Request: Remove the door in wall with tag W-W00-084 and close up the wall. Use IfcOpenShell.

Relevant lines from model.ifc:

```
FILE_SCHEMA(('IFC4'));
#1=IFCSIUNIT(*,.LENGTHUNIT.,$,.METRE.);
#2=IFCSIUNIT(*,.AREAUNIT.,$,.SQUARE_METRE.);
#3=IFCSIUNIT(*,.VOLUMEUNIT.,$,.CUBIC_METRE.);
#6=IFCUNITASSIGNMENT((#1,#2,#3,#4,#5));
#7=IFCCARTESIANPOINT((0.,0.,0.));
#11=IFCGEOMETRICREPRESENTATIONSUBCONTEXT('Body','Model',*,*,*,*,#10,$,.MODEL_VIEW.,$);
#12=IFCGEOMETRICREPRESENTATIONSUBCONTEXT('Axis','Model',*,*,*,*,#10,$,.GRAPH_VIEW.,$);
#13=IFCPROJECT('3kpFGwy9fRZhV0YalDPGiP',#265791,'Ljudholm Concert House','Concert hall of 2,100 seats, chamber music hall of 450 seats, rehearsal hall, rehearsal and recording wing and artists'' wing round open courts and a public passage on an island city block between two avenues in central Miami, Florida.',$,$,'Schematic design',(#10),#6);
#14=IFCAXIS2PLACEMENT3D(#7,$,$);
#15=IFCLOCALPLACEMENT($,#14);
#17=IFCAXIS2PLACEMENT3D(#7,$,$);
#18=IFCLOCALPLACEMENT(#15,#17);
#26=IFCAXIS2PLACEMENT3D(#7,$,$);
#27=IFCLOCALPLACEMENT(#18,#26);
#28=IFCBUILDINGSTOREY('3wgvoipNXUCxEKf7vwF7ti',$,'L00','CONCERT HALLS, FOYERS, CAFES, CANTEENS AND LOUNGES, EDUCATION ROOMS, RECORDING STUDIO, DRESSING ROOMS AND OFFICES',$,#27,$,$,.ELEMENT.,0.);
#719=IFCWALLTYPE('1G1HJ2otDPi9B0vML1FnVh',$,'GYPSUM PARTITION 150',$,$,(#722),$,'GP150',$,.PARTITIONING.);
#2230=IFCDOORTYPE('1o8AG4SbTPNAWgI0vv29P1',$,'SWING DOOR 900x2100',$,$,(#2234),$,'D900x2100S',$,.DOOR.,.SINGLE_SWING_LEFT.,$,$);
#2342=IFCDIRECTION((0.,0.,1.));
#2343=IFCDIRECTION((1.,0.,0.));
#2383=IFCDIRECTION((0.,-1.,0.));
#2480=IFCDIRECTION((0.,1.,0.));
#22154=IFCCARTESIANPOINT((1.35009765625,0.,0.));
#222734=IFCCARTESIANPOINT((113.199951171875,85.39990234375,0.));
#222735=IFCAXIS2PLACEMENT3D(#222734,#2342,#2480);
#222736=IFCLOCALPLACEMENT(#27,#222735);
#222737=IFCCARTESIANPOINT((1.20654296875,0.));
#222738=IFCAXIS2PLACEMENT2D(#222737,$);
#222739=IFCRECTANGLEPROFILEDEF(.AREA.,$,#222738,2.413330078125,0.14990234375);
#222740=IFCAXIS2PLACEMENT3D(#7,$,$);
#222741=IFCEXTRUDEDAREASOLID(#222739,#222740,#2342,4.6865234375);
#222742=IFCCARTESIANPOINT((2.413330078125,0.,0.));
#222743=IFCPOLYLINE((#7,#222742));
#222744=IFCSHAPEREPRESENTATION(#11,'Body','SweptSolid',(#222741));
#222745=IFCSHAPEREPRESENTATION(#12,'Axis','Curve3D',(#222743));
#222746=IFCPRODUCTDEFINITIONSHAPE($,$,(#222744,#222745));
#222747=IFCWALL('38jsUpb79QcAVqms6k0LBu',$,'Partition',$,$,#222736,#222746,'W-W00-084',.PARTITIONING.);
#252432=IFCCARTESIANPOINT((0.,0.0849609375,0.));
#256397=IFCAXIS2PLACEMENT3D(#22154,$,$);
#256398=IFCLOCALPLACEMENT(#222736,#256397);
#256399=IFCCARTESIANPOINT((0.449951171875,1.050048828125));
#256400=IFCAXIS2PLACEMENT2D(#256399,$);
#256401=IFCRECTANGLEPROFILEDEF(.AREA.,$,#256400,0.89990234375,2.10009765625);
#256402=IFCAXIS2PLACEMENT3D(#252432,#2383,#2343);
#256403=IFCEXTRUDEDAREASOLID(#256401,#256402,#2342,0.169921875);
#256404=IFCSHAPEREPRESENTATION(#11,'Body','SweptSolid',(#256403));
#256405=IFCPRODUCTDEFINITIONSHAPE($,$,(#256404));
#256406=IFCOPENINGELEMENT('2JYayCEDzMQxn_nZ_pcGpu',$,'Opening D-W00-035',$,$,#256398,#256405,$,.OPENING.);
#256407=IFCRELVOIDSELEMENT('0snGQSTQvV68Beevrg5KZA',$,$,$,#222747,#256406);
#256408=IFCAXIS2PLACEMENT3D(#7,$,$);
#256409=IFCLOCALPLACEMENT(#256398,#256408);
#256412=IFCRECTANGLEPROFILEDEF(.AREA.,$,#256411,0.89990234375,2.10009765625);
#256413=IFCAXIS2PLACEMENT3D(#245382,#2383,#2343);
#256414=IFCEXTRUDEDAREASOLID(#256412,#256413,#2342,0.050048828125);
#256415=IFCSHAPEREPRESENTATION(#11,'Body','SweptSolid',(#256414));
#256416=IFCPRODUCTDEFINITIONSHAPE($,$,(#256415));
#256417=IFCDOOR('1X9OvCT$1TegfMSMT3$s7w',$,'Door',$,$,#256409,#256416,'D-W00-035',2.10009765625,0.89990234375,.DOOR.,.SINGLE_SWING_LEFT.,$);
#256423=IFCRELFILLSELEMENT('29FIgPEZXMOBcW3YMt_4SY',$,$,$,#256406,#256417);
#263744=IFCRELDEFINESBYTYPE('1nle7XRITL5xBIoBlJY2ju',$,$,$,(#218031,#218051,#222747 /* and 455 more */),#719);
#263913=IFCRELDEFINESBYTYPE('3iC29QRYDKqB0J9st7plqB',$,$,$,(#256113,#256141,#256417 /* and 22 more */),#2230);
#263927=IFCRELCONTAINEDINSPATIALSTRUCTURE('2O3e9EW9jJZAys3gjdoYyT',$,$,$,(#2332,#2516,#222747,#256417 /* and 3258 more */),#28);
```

```python
import ifcopenshell
import ifcopenshell.api.feature
import ifcopenshell.api.root
import ifcopenshell.geom
import ifcopenshell.util.shape

model = ifcopenshell.open("model.ifc")
settings = ifcopenshell.geom.settings()


def volume(element):
    """Net volume in cubic metres, openings subtracted."""
    shape = ifcopenshell.geom.create_shape(settings, element)
    return ifcopenshell.util.shape.get_volume(shape.geometry)


door = model.by_guid("1X9OvCT$1TegfMSMT3$s7w")
opening = door.FillsVoids[0].RelatingOpeningElement
wall = opening.VoidsElements[0].RelatingBuildingElement
before = volume(wall)

ifcopenshell.api.root.remove_product(model, product=door)
ifcopenshell.api.feature.remove_feature(model, feature=opening)

after = volume(wall)

print(f"wall volume {before:.3f} -> {after:.3f} m3")

model.write("model_rev.ifc")
```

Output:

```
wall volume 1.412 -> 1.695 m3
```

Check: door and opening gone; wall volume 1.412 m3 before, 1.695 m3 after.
